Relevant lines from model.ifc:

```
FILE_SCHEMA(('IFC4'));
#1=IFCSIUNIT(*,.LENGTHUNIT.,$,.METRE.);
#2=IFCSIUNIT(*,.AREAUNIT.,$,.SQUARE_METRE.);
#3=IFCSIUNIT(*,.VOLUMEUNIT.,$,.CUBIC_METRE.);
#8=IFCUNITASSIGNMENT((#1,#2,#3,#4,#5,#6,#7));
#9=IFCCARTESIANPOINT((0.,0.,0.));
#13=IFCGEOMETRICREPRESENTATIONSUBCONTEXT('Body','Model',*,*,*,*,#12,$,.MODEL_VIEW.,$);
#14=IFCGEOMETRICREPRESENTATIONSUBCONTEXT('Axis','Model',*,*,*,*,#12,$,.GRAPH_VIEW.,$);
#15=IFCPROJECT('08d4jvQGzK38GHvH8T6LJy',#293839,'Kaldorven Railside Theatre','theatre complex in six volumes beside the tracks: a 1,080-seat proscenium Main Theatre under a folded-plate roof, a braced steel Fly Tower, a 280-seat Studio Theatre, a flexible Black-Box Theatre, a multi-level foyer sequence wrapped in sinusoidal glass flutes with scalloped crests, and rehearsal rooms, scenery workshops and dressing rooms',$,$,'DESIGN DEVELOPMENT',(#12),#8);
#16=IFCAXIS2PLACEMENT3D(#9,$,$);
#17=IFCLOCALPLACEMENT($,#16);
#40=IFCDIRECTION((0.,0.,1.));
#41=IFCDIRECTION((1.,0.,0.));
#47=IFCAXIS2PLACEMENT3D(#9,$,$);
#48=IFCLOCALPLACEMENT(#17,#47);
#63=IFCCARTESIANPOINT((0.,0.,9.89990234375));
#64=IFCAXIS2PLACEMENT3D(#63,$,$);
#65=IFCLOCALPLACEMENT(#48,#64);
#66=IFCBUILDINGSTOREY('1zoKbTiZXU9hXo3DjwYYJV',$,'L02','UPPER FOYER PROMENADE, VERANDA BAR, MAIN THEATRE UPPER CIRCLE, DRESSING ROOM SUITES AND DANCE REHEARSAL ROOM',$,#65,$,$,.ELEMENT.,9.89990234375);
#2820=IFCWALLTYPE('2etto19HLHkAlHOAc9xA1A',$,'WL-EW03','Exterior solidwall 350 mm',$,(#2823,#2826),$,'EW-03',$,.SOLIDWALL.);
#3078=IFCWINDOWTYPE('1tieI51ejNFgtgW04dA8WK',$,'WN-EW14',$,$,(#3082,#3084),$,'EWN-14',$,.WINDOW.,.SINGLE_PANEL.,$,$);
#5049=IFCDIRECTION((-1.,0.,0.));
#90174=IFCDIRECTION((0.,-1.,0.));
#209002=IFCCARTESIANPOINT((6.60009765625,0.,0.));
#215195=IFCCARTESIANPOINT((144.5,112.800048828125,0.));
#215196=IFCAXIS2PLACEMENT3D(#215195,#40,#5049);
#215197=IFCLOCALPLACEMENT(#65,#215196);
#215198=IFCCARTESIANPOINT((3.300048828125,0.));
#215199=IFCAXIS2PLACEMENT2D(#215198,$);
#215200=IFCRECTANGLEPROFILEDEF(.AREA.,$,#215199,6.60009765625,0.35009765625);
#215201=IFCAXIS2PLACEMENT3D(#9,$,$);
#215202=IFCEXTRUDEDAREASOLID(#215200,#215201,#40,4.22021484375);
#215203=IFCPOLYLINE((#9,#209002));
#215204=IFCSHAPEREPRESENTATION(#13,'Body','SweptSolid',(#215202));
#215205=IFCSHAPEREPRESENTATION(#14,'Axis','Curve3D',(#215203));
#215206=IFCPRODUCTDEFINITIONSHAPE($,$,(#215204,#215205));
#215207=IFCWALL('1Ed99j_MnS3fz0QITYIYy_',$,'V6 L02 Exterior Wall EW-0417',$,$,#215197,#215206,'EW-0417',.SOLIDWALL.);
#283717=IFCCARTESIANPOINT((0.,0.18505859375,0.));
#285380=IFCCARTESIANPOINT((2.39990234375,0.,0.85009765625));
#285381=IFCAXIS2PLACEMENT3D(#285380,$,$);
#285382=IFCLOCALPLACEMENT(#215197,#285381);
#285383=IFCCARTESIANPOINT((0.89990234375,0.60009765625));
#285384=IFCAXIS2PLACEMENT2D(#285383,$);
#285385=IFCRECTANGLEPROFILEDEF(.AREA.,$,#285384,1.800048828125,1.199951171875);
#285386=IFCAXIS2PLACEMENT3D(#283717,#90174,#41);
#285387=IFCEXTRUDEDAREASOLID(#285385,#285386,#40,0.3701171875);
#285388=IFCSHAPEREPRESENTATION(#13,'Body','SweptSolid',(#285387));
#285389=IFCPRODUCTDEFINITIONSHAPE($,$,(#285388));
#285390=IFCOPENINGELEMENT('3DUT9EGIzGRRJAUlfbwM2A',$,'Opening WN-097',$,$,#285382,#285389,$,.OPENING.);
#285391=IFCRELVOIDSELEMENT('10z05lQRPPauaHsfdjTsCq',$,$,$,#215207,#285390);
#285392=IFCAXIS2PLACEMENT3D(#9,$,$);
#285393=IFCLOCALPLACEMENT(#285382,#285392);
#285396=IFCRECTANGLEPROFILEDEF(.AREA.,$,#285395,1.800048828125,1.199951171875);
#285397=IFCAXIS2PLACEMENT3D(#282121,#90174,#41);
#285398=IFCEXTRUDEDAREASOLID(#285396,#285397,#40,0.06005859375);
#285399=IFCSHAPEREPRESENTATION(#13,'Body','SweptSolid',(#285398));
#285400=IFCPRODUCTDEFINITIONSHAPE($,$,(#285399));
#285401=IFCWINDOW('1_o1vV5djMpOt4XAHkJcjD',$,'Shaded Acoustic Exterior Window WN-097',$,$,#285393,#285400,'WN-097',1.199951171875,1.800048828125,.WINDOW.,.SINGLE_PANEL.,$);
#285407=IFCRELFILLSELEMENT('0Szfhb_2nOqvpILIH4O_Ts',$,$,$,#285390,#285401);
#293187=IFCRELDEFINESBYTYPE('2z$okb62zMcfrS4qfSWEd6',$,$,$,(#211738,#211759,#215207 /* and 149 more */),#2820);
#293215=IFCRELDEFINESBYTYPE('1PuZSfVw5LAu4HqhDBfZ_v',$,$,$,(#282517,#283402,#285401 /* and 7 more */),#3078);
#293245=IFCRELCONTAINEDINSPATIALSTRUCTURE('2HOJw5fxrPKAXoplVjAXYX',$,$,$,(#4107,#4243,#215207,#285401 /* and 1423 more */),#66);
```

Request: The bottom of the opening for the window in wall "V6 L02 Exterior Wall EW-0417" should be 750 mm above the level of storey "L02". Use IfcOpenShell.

```python
import numpy as np
import ifcopenshell
import ifcopenshell.api.geometry
import ifcopenshell.geom
import ifcopenshell.util.element
import ifcopenshell.util.placement
import ifcopenshell.util.shape
import ifcopenshell.util.unit

model = ifcopenshell.open("model.ifc")
unit_scale = ifcopenshell.util.unit.calculate_unit_scale(model)

window = model.by_id(285401)
opening = window.FillsVoids[0].RelatingOpeningElement
storey = ifcopenshell.util.element.get_container(window, ifc_class="IfcBuildingStorey")
level = ifcopenshell.util.placement.get_local_placement(storey.ObjectPlacement)[2, 3]

# The opening's origin need not be at the sill, so measure its lowest point.
shape = ifcopenshell.geom.create_shape(ifcopenshell.geom.settings(), opening)
bottom = ifcopenshell.util.shape.get_shape_bottom_elevation(shape, shape.geometry) / unit_scale
dz = level + 0.75 / unit_scale - bottom

shift = np.array([0.0, 0.0, dz])
# The window is placed relative to its opening, so it follows when the opening moves.
matrix = ifcopenshell.util.placement.get_local_placement(opening.ObjectPlacement)
matrix[:3, 3] += shift
ifcopenshell.api.geometry.edit_object_placement(
    model, product=opening, matrix=matrix, is_si=False, should_transform_children=True
)

print(f"moved by {dz * unit_scale:+.3f} m")

model.write("model_edited.ifc")
```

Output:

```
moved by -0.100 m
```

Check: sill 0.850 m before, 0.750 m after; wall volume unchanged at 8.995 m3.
